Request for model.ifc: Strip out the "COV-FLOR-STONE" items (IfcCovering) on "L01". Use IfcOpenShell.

First a look at what the model holds.

```python
import ifcopenshell
import ifcopenshell.util.element

model = ifcopenshell.open("model.ifc")
print(model.schema)
storey = next(s for s in model.by_type("IfcBuildingStorey") if s.Name == "L01")
coverings = [e for e in ifcopenshell.util.element.get_decomposition(storey) if e.is_a("IfcCovering")]
seen = {}
for e in coverings:
    element_type = ifcopenshell.util.element.get_type(e)
    name = element_type.Name if element_type not in (None, e) else None
    seen[name] = seen.get(name, 0) + 1
for name, count in sorted(seen.items(), key=str):
    print(count, "x", name)
```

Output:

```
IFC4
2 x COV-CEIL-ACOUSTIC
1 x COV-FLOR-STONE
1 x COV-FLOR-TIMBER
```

```python
import ifcopenshell
import ifcopenshell.api.root
import ifcopenshell.util.element

model = ifcopenshell.open("model.ifc")

storey = next(s for s in model.by_type("IfcBuildingStorey") if s.Name == "L01")
coverings = [e for e in ifcopenshell.util.element.get_decomposition(storey) if e.is_a("IfcCovering")]
targets = [e for e in coverings if (t := ifcopenshell.util.element.get_type(e)) not in (None, e) and t.Name == "COV-FLOR-STONE"]

for e in targets:
    ifcopenshell.api.root.remove_product(model, product=e)
print(len(targets), "removed")

model.write("model_updated.ifc")
```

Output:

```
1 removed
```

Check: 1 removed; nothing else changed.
